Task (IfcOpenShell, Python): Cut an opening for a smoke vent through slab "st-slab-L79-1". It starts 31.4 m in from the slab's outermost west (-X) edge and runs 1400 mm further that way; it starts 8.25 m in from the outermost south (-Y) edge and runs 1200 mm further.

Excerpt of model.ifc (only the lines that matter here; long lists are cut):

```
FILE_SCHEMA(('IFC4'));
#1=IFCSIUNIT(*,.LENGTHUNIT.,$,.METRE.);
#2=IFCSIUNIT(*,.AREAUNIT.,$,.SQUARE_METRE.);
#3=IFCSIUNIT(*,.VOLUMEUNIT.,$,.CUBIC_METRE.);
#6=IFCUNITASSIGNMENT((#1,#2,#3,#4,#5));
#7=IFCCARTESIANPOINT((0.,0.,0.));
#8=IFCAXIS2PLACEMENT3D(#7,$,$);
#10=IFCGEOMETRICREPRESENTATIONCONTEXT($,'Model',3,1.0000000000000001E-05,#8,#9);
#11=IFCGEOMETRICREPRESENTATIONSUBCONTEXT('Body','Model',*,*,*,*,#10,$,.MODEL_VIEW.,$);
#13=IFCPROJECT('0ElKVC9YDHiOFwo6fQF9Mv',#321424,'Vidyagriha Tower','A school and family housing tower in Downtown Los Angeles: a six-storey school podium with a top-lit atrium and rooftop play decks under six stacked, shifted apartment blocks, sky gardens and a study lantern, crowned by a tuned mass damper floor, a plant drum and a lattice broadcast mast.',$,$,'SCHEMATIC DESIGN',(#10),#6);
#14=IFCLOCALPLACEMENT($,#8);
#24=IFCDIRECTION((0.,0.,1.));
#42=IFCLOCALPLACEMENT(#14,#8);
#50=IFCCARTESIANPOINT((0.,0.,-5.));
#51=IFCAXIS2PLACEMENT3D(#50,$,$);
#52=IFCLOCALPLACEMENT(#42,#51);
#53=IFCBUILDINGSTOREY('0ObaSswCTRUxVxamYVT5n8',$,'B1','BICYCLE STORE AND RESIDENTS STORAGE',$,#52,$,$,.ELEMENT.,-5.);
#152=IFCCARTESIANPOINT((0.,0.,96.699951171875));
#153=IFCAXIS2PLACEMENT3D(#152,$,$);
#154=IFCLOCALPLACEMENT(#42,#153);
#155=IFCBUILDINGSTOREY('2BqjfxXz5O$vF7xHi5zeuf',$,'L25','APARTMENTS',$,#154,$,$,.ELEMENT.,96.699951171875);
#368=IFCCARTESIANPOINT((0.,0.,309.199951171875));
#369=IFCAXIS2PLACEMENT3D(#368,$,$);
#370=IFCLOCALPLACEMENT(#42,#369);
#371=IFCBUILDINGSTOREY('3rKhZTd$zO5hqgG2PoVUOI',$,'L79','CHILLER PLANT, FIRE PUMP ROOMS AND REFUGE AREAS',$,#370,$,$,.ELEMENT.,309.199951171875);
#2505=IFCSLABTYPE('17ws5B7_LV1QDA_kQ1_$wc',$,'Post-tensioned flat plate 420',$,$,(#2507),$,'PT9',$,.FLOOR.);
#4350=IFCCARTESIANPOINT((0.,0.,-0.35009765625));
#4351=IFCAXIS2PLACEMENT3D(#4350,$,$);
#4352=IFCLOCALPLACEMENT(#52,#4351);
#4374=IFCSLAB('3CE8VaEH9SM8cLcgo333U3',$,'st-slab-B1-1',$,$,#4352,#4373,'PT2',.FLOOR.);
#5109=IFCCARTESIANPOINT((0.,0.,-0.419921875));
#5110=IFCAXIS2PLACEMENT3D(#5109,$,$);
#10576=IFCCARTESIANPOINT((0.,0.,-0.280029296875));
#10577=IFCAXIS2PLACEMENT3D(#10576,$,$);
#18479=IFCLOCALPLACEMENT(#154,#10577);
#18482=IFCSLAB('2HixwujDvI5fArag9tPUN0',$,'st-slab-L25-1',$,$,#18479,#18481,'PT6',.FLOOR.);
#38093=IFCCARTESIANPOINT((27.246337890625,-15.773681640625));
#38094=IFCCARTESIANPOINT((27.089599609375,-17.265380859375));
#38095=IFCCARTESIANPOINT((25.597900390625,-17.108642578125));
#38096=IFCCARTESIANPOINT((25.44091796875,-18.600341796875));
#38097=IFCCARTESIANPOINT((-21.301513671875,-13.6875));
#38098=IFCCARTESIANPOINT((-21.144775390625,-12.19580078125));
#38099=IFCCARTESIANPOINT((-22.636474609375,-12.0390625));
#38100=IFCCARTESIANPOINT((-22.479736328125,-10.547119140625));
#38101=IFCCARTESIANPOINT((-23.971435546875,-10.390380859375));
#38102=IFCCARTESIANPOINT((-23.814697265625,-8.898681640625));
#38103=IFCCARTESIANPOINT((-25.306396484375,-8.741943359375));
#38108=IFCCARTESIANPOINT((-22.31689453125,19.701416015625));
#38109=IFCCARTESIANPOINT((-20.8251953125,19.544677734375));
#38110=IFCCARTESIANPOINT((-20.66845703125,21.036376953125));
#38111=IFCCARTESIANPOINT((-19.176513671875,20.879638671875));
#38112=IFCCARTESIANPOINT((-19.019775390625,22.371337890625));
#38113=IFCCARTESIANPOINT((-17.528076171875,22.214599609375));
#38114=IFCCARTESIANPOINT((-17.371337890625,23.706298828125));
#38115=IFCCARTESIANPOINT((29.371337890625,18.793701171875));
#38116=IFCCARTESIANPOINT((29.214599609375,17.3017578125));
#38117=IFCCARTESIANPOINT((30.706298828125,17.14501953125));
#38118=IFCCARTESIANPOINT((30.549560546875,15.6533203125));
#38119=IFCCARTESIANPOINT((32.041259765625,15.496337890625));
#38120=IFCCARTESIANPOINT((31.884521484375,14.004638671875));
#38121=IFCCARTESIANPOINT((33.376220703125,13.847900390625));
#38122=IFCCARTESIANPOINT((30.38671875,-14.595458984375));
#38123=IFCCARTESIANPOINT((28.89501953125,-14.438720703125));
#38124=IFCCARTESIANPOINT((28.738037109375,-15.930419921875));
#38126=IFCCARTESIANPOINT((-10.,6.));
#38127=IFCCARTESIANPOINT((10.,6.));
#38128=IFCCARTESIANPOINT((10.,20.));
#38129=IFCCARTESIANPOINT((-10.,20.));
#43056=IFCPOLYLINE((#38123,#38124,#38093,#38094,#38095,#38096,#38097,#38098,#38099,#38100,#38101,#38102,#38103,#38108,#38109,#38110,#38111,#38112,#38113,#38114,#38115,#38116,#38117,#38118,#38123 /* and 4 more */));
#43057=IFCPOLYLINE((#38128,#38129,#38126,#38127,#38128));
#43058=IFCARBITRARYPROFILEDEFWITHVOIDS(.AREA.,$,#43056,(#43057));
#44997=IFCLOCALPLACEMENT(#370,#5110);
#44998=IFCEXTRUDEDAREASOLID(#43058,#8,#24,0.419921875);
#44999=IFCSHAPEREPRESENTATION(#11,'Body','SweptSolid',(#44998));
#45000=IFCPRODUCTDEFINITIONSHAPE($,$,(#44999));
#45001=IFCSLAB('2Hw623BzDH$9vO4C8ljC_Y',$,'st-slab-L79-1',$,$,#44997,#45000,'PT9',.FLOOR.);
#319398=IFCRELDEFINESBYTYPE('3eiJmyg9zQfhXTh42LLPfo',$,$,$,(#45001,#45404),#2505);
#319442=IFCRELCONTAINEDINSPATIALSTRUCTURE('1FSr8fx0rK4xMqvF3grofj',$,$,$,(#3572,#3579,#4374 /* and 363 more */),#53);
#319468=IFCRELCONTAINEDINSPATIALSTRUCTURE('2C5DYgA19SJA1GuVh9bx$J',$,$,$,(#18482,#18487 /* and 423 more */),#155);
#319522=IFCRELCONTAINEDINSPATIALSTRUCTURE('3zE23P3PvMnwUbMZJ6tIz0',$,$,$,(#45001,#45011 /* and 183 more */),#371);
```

```python
import numpy as np
import ifcopenshell
import ifcopenshell.api.feature
import ifcopenshell.api.geometry
import ifcopenshell.api.root
import ifcopenshell.geom
import ifcopenshell.util.placement
import ifcopenshell.util.representation
import ifcopenshell.util.shape
import ifcopenshell.util.unit

model = ifcopenshell.open("model.ifc")
unit_scale = ifcopenshell.util.unit.calculate_unit_scale(model)
settings = ifcopenshell.geom.settings()


def volume(element):
    """Net volume in cubic metres, openings subtracted."""
    shape = ifcopenshell.geom.create_shape(settings, element)
    return ifcopenshell.util.shape.get_volume(shape.geometry)


slab = model.by_id(45001)
before = volume(slab)

# Extent in the slab's own axes, in metres. The edges named are its -X and -Y sides.
slab_shape = ifcopenshell.geom.create_shape(settings, slab)
vertices = ifcopenshell.util.shape.get_vertices(slab_shape.geometry)
x_min, y_min, bottom = vertices.min(axis=0)
top = vertices[:, 2].max()

opening = ifcopenshell.api.root.create_entity(model, ifc_class="IfcOpeningElement", name="Smoke vent opening", predefined_type="OPENING")
context = ifcopenshell.util.representation.get_context(model, "Model", "Body", "MODEL_VIEW")
width, depth = 1.4, 1.2
outline = [(0.0, 0.0), (width, 0.0), (width, depth), (0.0, depth), (0.0, 0.0)]
# Overshoot both faces by 50 mm so the cut is clean.
shape = ifcopenshell.api.geometry.add_slab_representation(
    model, context=context, depth=top - bottom + 0.1, polyline=outline
)
ifcopenshell.api.geometry.assign_representation(model, product=opening, representation=shape)

matrix = ifcopenshell.util.placement.get_local_placement(slab.ObjectPlacement)
matrix[:, 3] = matrix @ np.append(np.array([x_min + 31.4, y_min + 8.25, bottom - 0.05]) / unit_scale, 1.0)
ifcopenshell.api.geometry.edit_object_placement(model, product=opening, matrix=matrix, is_si=False)
ifcopenshell.api.feature.add_feature(model, feature=opening, element=slab)

after = volume(slab)

print(f"slab volume {before:.3f} -> {after:.3f} m3")

model.write("model_edited.ifc")
```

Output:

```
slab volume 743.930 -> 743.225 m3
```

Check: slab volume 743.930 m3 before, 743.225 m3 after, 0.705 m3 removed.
